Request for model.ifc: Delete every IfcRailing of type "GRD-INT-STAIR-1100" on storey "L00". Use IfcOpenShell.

First a look at what the model holds.

```python
import ifcopenshell
import ifcopenshell.util.element

model = ifcopenshell.open("model.ifc")
print(model.schema)
storey = next(s for s in model.by_type("IfcBuildingStorey") if s.Name == "L00")
railings = [e for e in ifcopenshell.util.element.get_decomposition(storey) if e.is_a("IfcRailing")]
seen = {}
for e in railings:
    element_type = ifcopenshell.util.element.get_type(e)
    name = element_type.Name if element_type not in (None, e) else None
    seen[name] = seen.get(name, 0) + 1
for name, count in sorted(seen.items(), key=str):
    print(count, "x", name)
```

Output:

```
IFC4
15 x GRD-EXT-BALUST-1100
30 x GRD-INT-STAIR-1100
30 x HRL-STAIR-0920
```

```python
import ifcopenshell
import ifcopenshell.api.root
import ifcopenshell.util.element

model = ifcopenshell.open("model.ifc")

storey = next(s for s in model.by_type("IfcBuildingStorey") if s.Name == "L00")
railings = [e for e in ifcopenshell.util.element.get_decomposition(storey) if e.is_a("IfcRailing")]
targets = [e for e in railings if (t := ifcopenshell.util.element.get_type(e)) not in (None, e) and t.Name == "GRD-INT-STAIR-1100"]

for e in targets:
    ifcopenshell.api.root.remove_product(model, product=e)
print(len(targets), "removed")

model.write("model_updated.ifc")
```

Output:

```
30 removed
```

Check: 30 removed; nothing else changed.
